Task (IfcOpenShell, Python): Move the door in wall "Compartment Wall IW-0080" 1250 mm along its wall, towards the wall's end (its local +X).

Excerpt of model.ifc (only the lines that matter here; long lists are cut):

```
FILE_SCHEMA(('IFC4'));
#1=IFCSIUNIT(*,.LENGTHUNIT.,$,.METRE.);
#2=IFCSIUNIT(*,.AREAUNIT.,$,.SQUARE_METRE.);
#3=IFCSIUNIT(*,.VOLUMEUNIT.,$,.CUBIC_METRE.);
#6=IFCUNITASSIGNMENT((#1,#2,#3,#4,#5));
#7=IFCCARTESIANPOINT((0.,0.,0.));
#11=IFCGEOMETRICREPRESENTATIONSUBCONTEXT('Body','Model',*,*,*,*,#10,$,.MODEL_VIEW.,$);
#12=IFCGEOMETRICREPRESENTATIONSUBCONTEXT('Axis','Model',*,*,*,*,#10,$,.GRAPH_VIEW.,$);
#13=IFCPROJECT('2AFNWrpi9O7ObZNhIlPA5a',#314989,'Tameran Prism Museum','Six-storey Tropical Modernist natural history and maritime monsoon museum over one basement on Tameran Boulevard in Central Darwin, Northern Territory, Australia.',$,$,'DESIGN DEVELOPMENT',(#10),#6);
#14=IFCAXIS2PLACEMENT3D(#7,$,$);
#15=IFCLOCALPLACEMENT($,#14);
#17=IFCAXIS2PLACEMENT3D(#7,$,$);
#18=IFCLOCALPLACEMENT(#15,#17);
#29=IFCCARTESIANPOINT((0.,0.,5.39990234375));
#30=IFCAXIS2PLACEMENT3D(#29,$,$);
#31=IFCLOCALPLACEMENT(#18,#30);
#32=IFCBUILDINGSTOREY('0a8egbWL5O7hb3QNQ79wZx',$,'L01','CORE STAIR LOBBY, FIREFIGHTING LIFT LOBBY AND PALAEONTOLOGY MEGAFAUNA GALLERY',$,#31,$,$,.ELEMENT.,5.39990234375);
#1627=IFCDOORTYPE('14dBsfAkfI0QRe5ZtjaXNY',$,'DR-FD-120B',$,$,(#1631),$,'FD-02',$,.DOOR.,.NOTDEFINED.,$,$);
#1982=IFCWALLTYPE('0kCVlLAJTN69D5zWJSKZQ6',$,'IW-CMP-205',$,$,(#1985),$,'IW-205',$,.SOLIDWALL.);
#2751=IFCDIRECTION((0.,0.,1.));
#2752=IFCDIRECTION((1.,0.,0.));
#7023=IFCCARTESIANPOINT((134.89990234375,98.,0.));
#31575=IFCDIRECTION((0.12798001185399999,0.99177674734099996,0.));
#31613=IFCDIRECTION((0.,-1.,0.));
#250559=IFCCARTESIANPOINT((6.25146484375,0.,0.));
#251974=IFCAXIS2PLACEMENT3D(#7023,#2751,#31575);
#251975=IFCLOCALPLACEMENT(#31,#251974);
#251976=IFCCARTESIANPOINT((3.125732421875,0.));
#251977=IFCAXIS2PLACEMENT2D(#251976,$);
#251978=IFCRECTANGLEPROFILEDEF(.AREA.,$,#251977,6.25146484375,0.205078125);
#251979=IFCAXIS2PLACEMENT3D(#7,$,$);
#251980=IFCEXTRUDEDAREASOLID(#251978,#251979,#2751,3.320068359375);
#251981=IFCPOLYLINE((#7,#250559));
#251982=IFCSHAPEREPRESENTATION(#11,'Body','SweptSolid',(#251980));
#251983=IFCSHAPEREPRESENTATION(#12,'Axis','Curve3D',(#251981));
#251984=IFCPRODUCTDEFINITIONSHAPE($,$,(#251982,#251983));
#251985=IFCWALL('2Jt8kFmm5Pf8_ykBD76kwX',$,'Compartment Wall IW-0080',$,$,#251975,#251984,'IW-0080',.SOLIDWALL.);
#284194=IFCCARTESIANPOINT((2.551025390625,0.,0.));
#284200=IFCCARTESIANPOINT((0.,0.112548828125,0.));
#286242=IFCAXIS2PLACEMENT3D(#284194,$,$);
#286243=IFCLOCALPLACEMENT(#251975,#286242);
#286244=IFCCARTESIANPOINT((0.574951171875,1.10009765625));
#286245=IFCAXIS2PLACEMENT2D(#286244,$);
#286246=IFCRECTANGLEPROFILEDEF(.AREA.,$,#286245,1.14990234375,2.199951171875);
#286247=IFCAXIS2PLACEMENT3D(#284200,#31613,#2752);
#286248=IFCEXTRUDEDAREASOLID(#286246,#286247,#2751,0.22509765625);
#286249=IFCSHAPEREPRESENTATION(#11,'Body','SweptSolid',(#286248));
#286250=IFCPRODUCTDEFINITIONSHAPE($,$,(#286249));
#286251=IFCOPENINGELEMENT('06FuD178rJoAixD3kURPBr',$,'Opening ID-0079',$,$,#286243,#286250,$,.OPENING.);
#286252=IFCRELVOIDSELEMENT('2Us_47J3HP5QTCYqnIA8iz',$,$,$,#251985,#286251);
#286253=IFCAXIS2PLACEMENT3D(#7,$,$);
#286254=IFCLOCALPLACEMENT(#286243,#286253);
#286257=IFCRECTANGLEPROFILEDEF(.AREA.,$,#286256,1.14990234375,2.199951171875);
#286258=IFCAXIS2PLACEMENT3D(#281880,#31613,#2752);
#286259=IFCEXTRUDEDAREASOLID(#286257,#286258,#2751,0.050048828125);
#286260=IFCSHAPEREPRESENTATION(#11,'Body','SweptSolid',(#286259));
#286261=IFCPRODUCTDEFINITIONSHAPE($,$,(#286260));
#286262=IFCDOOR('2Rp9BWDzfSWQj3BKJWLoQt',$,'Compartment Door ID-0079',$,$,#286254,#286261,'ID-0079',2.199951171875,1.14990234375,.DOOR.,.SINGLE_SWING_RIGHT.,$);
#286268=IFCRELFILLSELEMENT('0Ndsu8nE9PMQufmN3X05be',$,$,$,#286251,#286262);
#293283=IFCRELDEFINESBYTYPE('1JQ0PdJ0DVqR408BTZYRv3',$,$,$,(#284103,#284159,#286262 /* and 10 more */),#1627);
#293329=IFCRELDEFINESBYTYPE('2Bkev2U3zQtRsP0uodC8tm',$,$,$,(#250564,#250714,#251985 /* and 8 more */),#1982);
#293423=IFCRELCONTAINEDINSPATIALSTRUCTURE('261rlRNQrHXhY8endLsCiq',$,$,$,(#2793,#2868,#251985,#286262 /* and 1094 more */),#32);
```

```python
import ifcopenshell
import ifcopenshell.api.geometry
import ifcopenshell.util.placement

model = ifcopenshell.open("model.ifc")

door = model.by_guid("2Rp9BWDzfSWQj3BKJWLoQt")
opening = door.FillsVoids[0].RelatingOpeningElement
wall = opening.VoidsElements[0].RelatingBuildingElement

wall_matrix = ifcopenshell.util.placement.get_local_placement(wall.ObjectPlacement)
shift = wall_matrix[:3, 0] * 1.25
before = ifcopenshell.util.placement.get_local_placement(door.ObjectPlacement)[:3, 3].copy()

# The door is placed relative to its opening, so it follows when the opening moves.
matrix = ifcopenshell.util.placement.get_local_placement(opening.ObjectPlacement)
matrix[:3, 3] += shift
ifcopenshell.api.geometry.edit_object_placement(
    model, product=opening, matrix=matrix, is_si=False, should_transform_children=True
)

after = ifcopenshell.util.placement.get_local_placement(door.ObjectPlacement)[:3, 3]
print("door moved by", (after - before).round(3) + 0.0)

model.write("model_v2.ifc")
```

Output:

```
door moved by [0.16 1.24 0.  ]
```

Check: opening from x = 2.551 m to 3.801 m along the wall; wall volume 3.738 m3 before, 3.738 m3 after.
